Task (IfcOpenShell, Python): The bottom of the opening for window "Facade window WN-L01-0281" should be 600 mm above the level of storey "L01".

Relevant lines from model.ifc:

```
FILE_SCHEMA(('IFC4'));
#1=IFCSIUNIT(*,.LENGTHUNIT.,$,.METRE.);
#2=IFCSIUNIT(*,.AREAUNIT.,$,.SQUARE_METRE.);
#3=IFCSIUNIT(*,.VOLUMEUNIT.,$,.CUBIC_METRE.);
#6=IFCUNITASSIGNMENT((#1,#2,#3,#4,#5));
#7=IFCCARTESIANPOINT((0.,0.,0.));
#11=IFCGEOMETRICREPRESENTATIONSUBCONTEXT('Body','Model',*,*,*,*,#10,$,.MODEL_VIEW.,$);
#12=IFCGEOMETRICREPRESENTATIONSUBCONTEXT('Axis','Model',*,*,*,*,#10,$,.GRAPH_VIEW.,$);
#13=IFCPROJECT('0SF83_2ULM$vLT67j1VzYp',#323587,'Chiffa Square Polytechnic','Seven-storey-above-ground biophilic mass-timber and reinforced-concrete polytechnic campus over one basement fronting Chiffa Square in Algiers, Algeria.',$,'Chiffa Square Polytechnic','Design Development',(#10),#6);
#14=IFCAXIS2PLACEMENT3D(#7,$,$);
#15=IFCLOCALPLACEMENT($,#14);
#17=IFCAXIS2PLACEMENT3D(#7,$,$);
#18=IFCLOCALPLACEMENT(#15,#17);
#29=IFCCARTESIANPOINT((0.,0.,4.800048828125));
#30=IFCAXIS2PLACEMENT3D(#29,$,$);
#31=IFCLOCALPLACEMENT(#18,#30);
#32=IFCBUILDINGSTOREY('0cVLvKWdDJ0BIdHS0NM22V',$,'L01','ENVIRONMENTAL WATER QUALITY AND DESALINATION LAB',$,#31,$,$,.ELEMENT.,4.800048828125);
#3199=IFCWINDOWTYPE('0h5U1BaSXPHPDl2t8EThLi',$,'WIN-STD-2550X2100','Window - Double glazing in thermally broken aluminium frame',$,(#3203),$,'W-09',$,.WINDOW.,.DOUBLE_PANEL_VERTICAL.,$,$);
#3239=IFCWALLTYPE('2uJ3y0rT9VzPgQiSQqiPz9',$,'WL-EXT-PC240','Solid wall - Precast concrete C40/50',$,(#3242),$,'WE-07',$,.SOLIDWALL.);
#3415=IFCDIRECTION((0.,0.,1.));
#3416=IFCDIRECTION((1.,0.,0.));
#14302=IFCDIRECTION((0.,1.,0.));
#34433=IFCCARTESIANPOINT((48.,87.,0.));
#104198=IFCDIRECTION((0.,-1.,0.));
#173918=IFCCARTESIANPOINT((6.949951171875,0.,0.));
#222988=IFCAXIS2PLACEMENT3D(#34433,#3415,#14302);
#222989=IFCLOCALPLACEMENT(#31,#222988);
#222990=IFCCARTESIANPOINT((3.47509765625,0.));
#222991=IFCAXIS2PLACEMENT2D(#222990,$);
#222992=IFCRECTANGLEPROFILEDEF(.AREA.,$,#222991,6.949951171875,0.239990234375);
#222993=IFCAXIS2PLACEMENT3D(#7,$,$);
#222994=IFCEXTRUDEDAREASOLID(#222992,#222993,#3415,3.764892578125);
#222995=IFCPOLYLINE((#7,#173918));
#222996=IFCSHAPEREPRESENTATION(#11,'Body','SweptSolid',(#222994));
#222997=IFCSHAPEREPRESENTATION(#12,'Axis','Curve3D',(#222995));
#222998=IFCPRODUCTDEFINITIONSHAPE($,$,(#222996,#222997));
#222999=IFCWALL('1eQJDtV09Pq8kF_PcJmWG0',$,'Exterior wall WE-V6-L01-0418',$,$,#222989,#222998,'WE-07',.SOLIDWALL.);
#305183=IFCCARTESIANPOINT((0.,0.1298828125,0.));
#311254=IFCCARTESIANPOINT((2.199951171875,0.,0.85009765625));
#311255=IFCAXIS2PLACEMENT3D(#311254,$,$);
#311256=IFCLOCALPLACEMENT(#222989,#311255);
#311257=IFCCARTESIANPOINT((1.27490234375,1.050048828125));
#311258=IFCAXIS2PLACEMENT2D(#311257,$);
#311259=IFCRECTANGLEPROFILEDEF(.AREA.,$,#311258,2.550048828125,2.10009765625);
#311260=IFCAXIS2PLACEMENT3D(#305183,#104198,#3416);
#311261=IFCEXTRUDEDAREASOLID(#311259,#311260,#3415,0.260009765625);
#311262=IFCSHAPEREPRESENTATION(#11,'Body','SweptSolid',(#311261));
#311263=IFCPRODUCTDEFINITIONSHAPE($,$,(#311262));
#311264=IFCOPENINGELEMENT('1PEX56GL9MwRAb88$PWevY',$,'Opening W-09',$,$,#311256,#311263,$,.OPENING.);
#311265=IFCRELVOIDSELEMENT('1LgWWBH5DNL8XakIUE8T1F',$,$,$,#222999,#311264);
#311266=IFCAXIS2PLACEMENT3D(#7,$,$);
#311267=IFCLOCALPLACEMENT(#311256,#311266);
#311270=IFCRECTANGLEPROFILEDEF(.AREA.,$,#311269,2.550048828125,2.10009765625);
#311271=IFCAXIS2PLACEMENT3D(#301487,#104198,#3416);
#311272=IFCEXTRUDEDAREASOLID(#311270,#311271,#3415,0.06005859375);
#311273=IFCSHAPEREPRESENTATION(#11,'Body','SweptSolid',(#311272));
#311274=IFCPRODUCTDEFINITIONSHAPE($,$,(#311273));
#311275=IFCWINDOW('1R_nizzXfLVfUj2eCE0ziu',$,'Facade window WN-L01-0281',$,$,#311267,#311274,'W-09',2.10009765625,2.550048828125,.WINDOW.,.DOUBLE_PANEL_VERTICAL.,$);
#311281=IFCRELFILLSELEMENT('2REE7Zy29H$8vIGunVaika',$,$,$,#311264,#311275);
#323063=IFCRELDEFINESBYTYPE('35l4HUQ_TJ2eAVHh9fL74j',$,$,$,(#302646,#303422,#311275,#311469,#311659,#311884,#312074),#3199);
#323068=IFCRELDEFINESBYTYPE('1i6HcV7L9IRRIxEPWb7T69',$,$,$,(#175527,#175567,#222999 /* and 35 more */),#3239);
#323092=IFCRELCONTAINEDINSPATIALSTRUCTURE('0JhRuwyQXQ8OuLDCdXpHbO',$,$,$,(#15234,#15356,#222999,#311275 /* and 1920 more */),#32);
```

```python
import numpy as np
import ifcopenshell
import ifcopenshell.api.geometry
import ifcopenshell.geom
import ifcopenshell.util.element
import ifcopenshell.util.placement
import ifcopenshell.util.shape
import ifcopenshell.util.unit

model = ifcopenshell.open("model.ifc")
unit_scale = ifcopenshell.util.unit.calculate_unit_scale(model)

window = model.by_guid("1R_nizzXfLVfUj2eCE0ziu")
opening = window.FillsVoids[0].RelatingOpeningElement
storey = ifcopenshell.util.element.get_container(window, ifc_class="IfcBuildingStorey")
level = ifcopenshell.util.placement.get_local_placement(storey.ObjectPlacement)[2, 3]

# The opening's origin need not be at the sill, so measure its lowest point.
shape = ifcopenshell.geom.create_shape(ifcopenshell.geom.settings(), opening)
bottom = ifcopenshell.util.shape.get_shape_bottom_elevation(shape, shape.geometry) / unit_scale
dz = level + 0.6 - bottom

shift = np.array([0.0, 0.0, dz])
# The window is placed relative to its opening, so it follows when the opening moves.
matrix = ifcopenshell.util.placement.get_local_placement(opening.ObjectPlacement)
matrix[:3, 3] += shift
ifcopenshell.api.geometry.edit_object_placement(
    model, product=opening, matrix=matrix, is_si=False, should_transform_children=True
)

print(f"moved by {dz * unit_scale:+.3f} m")

model.write("model_updated.ifc")
```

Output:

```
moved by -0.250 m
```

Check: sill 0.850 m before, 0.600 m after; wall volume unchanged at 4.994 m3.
